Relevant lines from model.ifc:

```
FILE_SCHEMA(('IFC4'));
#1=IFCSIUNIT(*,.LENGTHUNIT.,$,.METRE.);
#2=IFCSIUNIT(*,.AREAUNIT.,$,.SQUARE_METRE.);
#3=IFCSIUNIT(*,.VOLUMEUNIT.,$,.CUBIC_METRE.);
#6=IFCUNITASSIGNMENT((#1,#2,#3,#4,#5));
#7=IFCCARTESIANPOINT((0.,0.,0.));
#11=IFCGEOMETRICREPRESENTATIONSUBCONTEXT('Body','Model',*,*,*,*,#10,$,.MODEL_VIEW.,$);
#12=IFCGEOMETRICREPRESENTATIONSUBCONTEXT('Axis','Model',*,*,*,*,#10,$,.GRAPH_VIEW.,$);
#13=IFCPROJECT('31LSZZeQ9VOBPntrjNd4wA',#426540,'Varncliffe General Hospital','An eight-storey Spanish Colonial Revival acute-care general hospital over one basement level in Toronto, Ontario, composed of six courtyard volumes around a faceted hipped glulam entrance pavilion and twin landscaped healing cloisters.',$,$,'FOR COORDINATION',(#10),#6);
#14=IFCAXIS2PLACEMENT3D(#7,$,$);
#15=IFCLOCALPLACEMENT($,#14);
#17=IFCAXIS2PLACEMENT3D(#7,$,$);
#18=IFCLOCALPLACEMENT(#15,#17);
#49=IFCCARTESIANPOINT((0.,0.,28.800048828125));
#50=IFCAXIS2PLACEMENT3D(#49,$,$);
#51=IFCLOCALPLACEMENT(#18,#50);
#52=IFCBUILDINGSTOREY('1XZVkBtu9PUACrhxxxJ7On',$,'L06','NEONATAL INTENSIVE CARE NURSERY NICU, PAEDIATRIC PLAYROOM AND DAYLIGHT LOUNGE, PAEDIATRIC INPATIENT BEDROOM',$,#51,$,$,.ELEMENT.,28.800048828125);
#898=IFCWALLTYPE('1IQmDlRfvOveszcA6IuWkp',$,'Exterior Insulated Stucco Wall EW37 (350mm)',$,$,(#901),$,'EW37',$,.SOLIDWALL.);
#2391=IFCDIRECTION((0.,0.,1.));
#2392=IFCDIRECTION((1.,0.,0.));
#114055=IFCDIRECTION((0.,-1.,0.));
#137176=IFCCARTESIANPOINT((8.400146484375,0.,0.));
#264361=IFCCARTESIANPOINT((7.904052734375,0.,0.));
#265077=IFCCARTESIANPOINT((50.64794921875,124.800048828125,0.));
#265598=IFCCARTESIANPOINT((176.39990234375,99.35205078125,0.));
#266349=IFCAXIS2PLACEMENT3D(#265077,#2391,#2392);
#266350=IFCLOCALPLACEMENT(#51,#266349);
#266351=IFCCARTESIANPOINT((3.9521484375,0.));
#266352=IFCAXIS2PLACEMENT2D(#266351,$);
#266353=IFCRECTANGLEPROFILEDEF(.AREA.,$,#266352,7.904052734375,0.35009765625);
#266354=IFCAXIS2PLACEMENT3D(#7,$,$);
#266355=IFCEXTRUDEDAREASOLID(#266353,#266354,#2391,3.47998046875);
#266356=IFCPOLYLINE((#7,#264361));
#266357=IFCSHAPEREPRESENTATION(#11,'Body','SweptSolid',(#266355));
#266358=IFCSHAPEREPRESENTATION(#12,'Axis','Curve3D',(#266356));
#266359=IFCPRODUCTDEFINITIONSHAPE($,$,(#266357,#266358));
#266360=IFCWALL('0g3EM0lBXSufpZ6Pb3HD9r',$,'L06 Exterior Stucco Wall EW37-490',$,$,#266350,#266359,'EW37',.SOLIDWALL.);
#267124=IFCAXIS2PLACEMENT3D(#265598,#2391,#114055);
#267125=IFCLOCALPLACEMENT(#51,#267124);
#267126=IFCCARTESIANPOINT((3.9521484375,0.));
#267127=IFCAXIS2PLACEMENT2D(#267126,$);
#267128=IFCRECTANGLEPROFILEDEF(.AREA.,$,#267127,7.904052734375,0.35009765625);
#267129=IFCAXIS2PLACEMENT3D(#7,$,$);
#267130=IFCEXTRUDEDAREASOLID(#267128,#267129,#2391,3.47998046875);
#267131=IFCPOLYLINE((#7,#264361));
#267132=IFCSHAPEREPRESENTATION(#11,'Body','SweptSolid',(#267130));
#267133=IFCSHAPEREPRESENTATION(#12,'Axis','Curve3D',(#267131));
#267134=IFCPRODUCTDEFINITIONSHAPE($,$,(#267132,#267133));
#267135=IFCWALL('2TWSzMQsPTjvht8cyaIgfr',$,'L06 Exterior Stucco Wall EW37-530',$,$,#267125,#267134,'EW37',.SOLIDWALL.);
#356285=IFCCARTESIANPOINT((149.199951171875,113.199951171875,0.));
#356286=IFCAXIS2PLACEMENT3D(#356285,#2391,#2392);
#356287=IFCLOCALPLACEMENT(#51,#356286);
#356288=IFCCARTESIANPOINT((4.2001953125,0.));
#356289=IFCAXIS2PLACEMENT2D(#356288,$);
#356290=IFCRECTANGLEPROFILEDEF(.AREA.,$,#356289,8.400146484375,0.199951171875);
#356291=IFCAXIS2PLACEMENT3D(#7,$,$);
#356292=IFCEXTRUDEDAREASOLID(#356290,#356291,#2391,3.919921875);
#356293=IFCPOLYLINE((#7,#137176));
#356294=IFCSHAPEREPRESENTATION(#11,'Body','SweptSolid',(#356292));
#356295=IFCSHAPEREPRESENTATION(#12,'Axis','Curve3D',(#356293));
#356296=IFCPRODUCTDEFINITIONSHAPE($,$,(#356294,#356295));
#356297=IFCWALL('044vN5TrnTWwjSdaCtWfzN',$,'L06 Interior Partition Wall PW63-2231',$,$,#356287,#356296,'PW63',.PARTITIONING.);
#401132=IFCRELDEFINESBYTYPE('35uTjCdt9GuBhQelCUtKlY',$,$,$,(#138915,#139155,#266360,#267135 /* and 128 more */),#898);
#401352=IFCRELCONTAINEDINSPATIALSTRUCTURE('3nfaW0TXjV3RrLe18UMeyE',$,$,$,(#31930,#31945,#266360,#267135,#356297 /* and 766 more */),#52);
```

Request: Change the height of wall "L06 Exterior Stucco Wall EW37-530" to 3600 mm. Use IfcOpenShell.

```python
import ifcopenshell
import ifcopenshell.geom
import ifcopenshell.util.representation
import ifcopenshell.util.shape
import ifcopenshell.util.unit

model = ifcopenshell.open("model.ifc")
unit_scale = ifcopenshell.util.unit.calculate_unit_scale(model)
settings = ifcopenshell.geom.settings()


def volume(element):
    """Net volume in cubic metres, openings subtracted."""
    shape = ifcopenshell.geom.create_shape(settings, element)
    return ifcopenshell.util.shape.get_volume(shape.geometry)


wall = model.by_guid("2TWSzMQsPTjvht8cyaIgfr")
before = volume(wall)

body = ifcopenshell.util.representation.get_representation(wall, "Model", "Body")
solid = body.Items[0]
old_height = solid.Depth
solid.Depth = 3.6 / unit_scale
after = volume(wall)

print(f"height {old_height:g} -> {solid.Depth:g}, volume {before:.3f} -> {after:.3f} m3")

model.write("model_edited.ifc")
```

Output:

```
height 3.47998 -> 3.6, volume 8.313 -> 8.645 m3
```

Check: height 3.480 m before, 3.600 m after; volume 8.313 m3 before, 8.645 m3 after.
